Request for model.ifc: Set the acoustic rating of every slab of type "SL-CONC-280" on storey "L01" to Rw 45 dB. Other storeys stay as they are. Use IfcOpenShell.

First a look at what the model holds.

```python
import ifcopenshell
import ifcopenshell.util.element

model = ifcopenshell.open("model.ifc")
print(model.schema)
storey = next(s for s in model.by_type("IfcBuildingStorey") if s.Name == "L01")
slabs = [e for e in ifcopenshell.util.element.get_decomposition(storey) if e.is_a("IfcSlab")]
seen = {}
for e in slabs:
    element_type = ifcopenshell.util.element.get_type(e)
    key = (element_type.Name if element_type != e and element_type else None, ifcopenshell.util.element.get_pset(e, "Pset_SlabCommon", "AcousticRating"))
    seen[key] = seen.get(key, 0) + 1
for (name, value), count in sorted(seen.items(), key=str):
    print(count, "x", name, "|", value)
```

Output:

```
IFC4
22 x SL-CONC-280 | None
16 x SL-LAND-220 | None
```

```python
import ifcopenshell
import ifcopenshell.api.pset
import ifcopenshell.util.element

model = ifcopenshell.open("model.ifc")

storey = next(s for s in model.by_type("IfcBuildingStorey") if s.Name == "L01")
slabs = [e for e in ifcopenshell.util.element.get_decomposition(storey) if e.is_a("IfcSlab")]

count = 0
for e in slabs:
    element_type = ifcopenshell.util.element.get_type(e)
    if element_type in (None, e) or element_type.Name != "SL-CONC-280":
        continue
    # add_pset returns the element's existing set when there is one.
    pset = ifcopenshell.api.pset.add_pset(model, product=e, name="Pset_SlabCommon")
    ifcopenshell.api.pset.edit_pset(model, pset=pset, properties={"AcousticRating": "Rw 45 dB"})
    count += 1

print(count, "slabs updated")

model.write("model_edited.ifc")
```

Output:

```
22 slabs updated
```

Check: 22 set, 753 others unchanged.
